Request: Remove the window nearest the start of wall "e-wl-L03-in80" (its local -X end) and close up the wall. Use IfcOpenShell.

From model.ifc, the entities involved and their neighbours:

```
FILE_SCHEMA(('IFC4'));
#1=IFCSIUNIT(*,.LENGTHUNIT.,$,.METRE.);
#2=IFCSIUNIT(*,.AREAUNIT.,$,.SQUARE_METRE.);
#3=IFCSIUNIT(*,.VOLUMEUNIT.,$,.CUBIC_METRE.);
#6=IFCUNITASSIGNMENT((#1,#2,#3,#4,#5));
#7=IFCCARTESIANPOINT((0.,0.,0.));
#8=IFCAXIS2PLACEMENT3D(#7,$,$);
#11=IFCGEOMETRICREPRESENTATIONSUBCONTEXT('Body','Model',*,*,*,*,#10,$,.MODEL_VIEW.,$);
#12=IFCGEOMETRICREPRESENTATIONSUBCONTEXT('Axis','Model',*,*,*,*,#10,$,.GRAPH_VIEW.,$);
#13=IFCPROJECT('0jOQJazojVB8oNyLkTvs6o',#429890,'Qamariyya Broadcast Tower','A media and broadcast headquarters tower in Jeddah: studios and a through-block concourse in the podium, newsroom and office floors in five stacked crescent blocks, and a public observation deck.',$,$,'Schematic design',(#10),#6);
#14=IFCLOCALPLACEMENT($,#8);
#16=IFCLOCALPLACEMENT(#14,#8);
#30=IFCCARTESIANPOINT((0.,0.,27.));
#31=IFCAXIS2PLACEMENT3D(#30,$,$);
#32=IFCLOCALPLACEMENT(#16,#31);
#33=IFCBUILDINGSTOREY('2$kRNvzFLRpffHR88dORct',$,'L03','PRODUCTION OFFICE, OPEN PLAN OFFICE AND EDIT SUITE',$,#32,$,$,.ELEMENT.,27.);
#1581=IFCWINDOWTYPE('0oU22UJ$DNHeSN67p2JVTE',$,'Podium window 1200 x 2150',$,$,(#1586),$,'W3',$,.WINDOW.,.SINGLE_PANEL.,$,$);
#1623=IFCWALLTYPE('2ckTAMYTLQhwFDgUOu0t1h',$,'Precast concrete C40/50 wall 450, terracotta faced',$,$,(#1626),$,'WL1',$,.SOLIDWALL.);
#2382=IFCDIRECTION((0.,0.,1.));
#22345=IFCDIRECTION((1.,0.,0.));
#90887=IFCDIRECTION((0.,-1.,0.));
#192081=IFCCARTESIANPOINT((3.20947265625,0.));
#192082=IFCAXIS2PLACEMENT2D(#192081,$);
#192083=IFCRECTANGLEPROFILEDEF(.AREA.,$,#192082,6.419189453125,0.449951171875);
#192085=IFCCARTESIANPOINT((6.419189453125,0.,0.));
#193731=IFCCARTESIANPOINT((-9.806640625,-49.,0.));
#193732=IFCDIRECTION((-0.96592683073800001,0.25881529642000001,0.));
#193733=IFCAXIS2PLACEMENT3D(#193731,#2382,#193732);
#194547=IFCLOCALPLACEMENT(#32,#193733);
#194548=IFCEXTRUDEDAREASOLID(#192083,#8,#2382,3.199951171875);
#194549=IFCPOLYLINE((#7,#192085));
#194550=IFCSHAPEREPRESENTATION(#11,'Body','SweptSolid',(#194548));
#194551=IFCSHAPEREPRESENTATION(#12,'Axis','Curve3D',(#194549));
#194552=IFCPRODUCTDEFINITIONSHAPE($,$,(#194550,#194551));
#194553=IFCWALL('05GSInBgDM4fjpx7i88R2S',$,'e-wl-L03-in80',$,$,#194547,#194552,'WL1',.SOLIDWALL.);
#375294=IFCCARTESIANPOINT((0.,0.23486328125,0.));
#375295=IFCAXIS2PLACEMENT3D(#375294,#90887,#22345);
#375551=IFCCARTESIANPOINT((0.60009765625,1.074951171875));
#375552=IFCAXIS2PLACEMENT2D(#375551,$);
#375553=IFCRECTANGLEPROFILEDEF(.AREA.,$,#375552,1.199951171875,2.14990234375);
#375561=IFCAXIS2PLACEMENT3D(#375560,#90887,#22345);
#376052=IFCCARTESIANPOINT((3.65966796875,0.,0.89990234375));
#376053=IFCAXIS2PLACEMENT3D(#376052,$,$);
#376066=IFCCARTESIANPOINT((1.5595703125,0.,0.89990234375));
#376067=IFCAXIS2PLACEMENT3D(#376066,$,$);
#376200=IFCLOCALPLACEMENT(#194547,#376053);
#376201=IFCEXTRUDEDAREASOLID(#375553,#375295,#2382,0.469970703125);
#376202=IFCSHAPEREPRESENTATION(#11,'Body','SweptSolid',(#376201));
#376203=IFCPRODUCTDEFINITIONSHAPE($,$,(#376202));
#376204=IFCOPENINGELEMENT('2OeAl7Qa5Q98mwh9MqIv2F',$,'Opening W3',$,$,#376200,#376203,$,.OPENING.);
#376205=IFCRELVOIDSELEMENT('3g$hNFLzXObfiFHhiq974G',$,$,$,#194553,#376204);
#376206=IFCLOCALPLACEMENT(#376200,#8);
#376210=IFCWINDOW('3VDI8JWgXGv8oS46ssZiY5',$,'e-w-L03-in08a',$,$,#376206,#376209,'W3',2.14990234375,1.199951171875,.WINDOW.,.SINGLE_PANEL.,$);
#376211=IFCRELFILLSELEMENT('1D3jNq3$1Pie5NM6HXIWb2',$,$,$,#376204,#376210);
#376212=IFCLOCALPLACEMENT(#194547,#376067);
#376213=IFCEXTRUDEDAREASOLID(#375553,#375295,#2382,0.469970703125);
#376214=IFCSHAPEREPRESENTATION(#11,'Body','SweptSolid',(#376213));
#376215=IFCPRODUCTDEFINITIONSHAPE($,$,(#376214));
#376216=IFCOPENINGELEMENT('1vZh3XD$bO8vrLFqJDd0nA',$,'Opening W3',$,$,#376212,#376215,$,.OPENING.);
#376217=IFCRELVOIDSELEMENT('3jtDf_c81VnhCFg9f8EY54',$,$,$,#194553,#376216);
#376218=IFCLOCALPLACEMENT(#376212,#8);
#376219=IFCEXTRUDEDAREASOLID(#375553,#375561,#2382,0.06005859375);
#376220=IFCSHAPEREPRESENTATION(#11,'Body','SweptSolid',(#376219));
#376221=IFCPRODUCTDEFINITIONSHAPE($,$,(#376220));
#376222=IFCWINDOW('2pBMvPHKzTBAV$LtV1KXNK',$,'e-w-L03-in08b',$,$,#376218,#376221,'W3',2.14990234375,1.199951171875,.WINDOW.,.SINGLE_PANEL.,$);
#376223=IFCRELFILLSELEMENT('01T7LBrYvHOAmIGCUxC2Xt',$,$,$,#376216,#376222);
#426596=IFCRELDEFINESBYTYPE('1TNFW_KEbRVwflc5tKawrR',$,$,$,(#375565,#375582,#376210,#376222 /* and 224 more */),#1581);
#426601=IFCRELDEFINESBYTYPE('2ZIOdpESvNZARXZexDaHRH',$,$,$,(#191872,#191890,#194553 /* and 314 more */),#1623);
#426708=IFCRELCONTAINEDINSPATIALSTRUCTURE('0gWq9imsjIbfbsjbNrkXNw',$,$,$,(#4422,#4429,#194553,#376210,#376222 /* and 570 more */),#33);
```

```python
import ifcopenshell
import ifcopenshell.api.feature
import ifcopenshell.api.root
import ifcopenshell.geom
import ifcopenshell.util.shape

model = ifcopenshell.open("model.ifc")
settings = ifcopenshell.geom.settings()


def volume(element):
    """Net volume in cubic metres, openings subtracted."""
    shape = ifcopenshell.geom.create_shape(settings, element)
    return ifcopenshell.util.shape.get_volume(shape.geometry)


window = model.by_id(376222)
opening = window.FillsVoids[0].RelatingOpeningElement
wall = opening.VoidsElements[0].RelatingBuildingElement
before = volume(wall)

ifcopenshell.api.root.remove_product(model, product=window)
ifcopenshell.api.feature.remove_feature(model, feature=opening)

after = volume(wall)

print(f"wall volume {before:.3f} -> {after:.3f} m3")

model.write("model_edited.ifc")
```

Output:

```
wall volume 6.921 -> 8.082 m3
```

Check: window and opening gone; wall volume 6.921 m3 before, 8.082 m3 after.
